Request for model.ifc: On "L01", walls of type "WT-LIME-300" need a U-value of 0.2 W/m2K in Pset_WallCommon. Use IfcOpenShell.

First a look at what the model holds.

```python
import ifcopenshell
import ifcopenshell.util.element

model = ifcopenshell.open("model.ifc")
print(model.schema)
storey = next(s for s in model.by_type("IfcBuildingStorey") if s.Name == "L01")
walls = [e for e in ifcopenshell.util.element.get_decomposition(storey) if e.is_a("IfcWall")]
seen = {}
for e in walls:
    element_type = ifcopenshell.util.element.get_type(e)
    key = (element_type.Name if element_type != e and element_type else None, ifcopenshell.util.element.get_pset(e, "Pset_WallCommon", "ThermalTransmittance"))
    seen[key] = seen.get(key, 0) + 1
for (name, value), count in sorted(seen.items(), key=str):
    print(count, "x", name, "|", value)
```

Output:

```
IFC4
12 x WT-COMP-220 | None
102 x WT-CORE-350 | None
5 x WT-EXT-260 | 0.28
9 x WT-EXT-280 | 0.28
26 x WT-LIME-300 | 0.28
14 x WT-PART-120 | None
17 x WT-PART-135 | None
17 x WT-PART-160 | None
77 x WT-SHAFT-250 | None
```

```python
import ifcopenshell
import ifcopenshell.api.pset
import ifcopenshell.util.element

model = ifcopenshell.open("model.ifc")

storey = next(s for s in model.by_type("IfcBuildingStorey") if s.Name == "L01")
walls = [e for e in ifcopenshell.util.element.get_decomposition(storey) if e.is_a("IfcWall")]

count = 0
for e in walls:
    element_type = ifcopenshell.util.element.get_type(e)
    if element_type in (None, e) or element_type.Name != "WT-LIME-300":
        continue
    # add_pset returns the element's existing set when there is one.
    pset = ifcopenshell.api.pset.add_pset(model, product=e, name="Pset_WallCommon")
    ifcopenshell.api.pset.edit_pset(model, pset=pset, properties={"ThermalTransmittance": 0.2})
    count += 1

print(count, "walls updated")

model.write("model_rev.ifc")
```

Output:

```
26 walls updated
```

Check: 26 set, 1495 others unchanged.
